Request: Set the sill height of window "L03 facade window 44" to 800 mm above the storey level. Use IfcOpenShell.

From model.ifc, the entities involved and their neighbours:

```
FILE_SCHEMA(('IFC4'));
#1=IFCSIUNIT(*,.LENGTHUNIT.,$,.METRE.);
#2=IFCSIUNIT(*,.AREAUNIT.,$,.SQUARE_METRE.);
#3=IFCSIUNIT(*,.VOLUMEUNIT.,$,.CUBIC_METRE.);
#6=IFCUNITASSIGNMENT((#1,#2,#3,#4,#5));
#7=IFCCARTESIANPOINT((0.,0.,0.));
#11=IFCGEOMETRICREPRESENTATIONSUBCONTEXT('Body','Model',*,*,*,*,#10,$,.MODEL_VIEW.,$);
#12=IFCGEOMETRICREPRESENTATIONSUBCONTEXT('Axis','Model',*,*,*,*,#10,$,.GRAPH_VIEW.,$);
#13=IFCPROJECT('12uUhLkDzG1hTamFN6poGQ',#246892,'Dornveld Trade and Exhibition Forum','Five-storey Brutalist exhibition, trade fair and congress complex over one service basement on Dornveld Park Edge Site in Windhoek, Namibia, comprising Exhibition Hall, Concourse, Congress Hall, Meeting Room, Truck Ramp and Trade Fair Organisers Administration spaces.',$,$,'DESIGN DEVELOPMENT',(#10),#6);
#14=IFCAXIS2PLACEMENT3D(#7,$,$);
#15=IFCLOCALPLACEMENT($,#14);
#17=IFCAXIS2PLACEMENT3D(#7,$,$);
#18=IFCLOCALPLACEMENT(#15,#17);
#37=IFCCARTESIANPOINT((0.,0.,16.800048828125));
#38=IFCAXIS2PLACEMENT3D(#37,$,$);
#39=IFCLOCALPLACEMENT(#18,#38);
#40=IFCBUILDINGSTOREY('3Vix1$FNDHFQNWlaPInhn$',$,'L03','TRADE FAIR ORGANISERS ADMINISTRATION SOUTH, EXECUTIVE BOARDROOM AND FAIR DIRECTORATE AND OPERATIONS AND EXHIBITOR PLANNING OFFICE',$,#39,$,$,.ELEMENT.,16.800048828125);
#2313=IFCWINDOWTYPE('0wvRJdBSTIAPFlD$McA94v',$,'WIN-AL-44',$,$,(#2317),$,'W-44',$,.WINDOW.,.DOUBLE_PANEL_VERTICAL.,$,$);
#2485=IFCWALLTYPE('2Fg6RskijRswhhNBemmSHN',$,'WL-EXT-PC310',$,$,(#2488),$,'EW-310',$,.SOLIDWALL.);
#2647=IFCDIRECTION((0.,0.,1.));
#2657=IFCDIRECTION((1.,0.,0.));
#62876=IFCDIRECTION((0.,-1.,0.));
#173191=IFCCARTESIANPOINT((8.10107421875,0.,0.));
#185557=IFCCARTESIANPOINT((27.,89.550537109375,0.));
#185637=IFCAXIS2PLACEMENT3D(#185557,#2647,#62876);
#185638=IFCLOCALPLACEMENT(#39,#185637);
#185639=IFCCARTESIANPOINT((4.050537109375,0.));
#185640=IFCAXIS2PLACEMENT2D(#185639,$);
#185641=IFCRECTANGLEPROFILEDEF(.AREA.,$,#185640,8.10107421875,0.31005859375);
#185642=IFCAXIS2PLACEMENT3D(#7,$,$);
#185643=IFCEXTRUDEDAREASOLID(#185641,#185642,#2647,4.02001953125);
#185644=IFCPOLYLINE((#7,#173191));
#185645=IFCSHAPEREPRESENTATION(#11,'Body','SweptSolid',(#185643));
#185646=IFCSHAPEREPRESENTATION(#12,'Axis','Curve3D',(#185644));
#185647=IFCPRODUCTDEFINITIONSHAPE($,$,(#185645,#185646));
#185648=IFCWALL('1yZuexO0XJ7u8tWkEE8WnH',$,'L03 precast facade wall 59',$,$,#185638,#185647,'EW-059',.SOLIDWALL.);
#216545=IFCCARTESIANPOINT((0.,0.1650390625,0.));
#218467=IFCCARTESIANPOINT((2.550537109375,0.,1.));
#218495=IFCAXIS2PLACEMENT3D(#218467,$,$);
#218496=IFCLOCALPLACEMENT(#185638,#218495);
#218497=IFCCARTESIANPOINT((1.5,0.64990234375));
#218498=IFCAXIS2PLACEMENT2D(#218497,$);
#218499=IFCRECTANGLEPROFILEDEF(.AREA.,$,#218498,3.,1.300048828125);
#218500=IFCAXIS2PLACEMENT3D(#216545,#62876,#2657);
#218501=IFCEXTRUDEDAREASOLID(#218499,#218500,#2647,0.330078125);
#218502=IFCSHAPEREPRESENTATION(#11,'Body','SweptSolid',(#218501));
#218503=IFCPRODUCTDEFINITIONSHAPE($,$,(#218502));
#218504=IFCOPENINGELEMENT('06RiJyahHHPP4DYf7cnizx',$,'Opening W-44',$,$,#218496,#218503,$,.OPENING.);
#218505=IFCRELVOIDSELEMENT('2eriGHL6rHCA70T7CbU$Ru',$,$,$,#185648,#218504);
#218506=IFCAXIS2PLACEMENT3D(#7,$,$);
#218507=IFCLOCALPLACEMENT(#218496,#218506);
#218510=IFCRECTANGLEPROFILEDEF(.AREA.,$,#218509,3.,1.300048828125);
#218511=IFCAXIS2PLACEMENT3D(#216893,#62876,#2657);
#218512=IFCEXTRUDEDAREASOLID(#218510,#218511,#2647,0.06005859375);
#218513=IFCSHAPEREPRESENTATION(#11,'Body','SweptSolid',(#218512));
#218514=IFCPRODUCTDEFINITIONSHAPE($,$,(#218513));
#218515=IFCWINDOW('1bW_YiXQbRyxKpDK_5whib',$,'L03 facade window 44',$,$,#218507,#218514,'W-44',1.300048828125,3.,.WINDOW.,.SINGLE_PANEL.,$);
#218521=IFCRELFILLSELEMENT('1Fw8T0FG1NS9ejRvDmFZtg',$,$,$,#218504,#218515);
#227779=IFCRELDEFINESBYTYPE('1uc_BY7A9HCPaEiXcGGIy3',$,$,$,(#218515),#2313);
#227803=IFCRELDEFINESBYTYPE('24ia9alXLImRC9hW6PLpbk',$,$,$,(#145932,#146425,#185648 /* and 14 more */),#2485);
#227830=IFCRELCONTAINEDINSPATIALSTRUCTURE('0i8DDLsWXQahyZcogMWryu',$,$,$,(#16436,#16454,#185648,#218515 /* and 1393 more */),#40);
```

```python
import numpy as np
import ifcopenshell
import ifcopenshell.api.geometry
import ifcopenshell.geom
import ifcopenshell.util.element
import ifcopenshell.util.placement
import ifcopenshell.util.shape
import ifcopenshell.util.unit

model = ifcopenshell.open("model.ifc")
unit_scale = ifcopenshell.util.unit.calculate_unit_scale(model)

window = model.by_guid("1bW_YiXQbRyxKpDK_5whib")
opening = window.FillsVoids[0].RelatingOpeningElement
storey = ifcopenshell.util.element.get_container(window, ifc_class="IfcBuildingStorey")
level = ifcopenshell.util.placement.get_local_placement(storey.ObjectPlacement)[2, 3]

# The opening's origin need not be at the sill, so measure its lowest point.
shape = ifcopenshell.geom.create_shape(ifcopenshell.geom.settings(), opening)
bottom = ifcopenshell.util.shape.get_shape_bottom_elevation(shape, shape.geometry) / unit_scale
dz = level + 0.8 / unit_scale - bottom

shift = np.array([0.0, 0.0, dz])
# The window is placed relative to its opening, so it follows when the opening moves.
matrix = ifcopenshell.util.placement.get_local_placement(opening.ObjectPlacement)
matrix[:3, 3] += shift
ifcopenshell.api.geometry.edit_object_placement(
    model, product=opening, matrix=matrix, is_si=False, should_transform_children=True
)

print(f"moved by {dz * unit_scale:+.3f} m")

model.write("model_rev.ifc")
```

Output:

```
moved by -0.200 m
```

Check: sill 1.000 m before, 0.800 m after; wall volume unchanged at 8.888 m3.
